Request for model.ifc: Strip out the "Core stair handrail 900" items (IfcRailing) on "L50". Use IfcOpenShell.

First a look at what the model holds.

```python
import ifcopenshell
import ifcopenshell.util.element

model = ifcopenshell.open("model.ifc")
print(model.schema)
storey = next(s for s in model.by_type("IfcBuildingStorey") if s.Name == "L50")
railings = [e for e in ifcopenshell.util.element.get_decomposition(storey) if e.is_a("IfcRailing")]
seen = {}
for e in railings:
    element_type = ifcopenshell.util.element.get_type(e)
    name = element_type.Name if element_type not in (None, e) else None
    seen[name] = seen.get(name, 0) + 1
for name, count in sorted(seen.items(), key=str):
    print(count, "x", name)
```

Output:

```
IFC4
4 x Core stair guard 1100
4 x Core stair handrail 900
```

```python
import ifcopenshell
import ifcopenshell.api.root
import ifcopenshell.util.element

model = ifcopenshell.open("model.ifc")

storey = next(s for s in model.by_type("IfcBuildingStorey") if s.Name == "L50")
railings = [e for e in ifcopenshell.util.element.get_decomposition(storey) if e.is_a("IfcRailing")]
targets = [e for e in railings if (t := ifcopenshell.util.element.get_type(e)) not in (None, e) and t.Name == "Core stair handrail 900"]

for e in targets:
    ifcopenshell.api.root.remove_product(model, product=e)
print(len(targets), "removed")

model.write("model_edited.ifc")
```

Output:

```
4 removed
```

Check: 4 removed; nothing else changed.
